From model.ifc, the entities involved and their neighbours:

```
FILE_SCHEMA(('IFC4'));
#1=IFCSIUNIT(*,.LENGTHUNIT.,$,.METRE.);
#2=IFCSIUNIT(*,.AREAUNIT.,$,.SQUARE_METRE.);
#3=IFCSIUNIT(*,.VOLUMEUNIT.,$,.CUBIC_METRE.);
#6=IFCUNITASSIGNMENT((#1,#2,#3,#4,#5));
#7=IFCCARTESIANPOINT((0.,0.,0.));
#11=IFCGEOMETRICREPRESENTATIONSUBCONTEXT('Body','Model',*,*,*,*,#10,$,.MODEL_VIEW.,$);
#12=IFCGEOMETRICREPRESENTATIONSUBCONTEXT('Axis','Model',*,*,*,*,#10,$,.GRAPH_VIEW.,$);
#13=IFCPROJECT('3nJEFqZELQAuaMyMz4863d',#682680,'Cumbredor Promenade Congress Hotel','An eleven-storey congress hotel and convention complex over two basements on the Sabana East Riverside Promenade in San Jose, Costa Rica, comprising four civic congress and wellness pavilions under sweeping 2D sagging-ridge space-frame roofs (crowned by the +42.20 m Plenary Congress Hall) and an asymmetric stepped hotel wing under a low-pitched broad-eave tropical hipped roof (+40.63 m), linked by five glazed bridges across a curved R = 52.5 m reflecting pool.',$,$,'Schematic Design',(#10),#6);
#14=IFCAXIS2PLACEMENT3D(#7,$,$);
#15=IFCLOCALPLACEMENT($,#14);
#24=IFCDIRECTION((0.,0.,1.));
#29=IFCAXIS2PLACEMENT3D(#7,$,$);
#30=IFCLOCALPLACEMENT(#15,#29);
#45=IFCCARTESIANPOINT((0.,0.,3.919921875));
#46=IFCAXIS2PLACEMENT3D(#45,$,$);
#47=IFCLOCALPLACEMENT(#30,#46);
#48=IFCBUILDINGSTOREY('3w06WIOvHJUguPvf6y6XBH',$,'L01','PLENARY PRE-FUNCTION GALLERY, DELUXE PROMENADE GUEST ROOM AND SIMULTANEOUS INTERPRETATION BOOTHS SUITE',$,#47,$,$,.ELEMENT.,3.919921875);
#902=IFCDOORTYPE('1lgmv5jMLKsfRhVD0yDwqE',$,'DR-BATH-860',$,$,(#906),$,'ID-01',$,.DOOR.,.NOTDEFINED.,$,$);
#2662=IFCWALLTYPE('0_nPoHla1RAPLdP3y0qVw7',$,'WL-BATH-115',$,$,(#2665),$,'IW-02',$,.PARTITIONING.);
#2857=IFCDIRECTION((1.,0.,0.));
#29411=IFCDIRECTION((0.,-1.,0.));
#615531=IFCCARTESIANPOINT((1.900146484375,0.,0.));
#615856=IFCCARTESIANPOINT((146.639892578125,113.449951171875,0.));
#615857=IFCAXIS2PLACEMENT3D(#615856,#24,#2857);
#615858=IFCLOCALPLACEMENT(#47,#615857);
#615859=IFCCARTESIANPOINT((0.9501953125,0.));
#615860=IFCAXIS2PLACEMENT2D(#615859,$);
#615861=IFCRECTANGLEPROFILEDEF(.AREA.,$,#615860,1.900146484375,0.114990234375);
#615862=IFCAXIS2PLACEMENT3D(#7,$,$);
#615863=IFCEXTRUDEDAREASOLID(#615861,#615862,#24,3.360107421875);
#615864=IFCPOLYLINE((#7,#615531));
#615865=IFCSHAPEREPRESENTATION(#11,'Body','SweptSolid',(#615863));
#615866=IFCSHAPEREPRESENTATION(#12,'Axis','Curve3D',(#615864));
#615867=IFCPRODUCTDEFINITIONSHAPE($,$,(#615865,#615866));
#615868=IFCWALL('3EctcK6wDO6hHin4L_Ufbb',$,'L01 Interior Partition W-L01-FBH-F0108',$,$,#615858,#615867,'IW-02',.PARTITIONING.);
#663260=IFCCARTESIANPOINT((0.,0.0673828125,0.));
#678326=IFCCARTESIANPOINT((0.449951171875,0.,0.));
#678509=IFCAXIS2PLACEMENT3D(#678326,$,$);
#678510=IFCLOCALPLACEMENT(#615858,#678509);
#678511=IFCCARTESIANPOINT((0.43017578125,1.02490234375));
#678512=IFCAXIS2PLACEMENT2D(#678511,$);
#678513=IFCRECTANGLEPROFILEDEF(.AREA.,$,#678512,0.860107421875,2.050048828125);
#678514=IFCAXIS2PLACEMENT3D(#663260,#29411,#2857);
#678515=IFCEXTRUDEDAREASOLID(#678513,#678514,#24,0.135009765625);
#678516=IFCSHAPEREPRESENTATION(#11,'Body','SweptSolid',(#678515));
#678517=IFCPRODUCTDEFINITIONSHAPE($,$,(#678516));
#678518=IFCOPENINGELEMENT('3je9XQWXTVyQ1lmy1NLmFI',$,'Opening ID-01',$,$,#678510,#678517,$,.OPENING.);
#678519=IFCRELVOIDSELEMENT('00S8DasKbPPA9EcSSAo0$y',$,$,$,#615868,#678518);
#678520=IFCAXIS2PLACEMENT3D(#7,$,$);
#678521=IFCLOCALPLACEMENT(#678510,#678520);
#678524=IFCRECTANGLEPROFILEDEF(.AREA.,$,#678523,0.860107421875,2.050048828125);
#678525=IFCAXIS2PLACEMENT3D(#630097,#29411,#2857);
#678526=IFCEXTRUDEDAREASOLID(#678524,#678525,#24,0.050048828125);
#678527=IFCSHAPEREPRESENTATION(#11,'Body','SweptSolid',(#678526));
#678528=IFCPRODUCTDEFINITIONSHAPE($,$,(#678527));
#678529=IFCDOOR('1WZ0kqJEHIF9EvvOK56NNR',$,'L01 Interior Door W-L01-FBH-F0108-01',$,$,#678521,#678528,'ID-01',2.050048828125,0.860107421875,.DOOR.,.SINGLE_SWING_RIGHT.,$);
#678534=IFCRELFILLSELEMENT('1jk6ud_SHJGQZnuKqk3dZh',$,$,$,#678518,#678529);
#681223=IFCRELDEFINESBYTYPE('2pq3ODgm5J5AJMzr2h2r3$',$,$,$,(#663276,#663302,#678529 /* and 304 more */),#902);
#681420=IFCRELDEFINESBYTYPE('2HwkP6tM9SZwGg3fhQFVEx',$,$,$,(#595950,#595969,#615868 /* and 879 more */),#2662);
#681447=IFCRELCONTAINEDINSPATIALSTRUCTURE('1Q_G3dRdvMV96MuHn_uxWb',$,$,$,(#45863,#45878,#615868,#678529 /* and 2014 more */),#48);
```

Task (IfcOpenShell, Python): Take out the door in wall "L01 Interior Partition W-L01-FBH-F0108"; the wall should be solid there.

```python
import ifcopenshell
import ifcopenshell.api.feature
import ifcopenshell.api.root
import ifcopenshell.geom
import ifcopenshell.util.shape

model = ifcopenshell.open("model.ifc")
settings = ifcopenshell.geom.settings()


def volume(element):
    """Net volume in cubic metres, openings subtracted."""
    shape = ifcopenshell.geom.create_shape(settings, element)
    return ifcopenshell.util.shape.get_volume(shape.geometry)


door = model.by_guid("1WZ0kqJEHIF9EvvOK56NNR")
opening = door.FillsVoids[0].RelatingOpeningElement
wall = opening.VoidsElements[0].RelatingBuildingElement
before = volume(wall)

ifcopenshell.api.root.remove_product(model, product=door)
ifcopenshell.api.feature.remove_feature(model, feature=opening)

after = volume(wall)

print(f"wall volume {before:.3f} -> {after:.3f} m3")

model.write("model_updated.ifc")
```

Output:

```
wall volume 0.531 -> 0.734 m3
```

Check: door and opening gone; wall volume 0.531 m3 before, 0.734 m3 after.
